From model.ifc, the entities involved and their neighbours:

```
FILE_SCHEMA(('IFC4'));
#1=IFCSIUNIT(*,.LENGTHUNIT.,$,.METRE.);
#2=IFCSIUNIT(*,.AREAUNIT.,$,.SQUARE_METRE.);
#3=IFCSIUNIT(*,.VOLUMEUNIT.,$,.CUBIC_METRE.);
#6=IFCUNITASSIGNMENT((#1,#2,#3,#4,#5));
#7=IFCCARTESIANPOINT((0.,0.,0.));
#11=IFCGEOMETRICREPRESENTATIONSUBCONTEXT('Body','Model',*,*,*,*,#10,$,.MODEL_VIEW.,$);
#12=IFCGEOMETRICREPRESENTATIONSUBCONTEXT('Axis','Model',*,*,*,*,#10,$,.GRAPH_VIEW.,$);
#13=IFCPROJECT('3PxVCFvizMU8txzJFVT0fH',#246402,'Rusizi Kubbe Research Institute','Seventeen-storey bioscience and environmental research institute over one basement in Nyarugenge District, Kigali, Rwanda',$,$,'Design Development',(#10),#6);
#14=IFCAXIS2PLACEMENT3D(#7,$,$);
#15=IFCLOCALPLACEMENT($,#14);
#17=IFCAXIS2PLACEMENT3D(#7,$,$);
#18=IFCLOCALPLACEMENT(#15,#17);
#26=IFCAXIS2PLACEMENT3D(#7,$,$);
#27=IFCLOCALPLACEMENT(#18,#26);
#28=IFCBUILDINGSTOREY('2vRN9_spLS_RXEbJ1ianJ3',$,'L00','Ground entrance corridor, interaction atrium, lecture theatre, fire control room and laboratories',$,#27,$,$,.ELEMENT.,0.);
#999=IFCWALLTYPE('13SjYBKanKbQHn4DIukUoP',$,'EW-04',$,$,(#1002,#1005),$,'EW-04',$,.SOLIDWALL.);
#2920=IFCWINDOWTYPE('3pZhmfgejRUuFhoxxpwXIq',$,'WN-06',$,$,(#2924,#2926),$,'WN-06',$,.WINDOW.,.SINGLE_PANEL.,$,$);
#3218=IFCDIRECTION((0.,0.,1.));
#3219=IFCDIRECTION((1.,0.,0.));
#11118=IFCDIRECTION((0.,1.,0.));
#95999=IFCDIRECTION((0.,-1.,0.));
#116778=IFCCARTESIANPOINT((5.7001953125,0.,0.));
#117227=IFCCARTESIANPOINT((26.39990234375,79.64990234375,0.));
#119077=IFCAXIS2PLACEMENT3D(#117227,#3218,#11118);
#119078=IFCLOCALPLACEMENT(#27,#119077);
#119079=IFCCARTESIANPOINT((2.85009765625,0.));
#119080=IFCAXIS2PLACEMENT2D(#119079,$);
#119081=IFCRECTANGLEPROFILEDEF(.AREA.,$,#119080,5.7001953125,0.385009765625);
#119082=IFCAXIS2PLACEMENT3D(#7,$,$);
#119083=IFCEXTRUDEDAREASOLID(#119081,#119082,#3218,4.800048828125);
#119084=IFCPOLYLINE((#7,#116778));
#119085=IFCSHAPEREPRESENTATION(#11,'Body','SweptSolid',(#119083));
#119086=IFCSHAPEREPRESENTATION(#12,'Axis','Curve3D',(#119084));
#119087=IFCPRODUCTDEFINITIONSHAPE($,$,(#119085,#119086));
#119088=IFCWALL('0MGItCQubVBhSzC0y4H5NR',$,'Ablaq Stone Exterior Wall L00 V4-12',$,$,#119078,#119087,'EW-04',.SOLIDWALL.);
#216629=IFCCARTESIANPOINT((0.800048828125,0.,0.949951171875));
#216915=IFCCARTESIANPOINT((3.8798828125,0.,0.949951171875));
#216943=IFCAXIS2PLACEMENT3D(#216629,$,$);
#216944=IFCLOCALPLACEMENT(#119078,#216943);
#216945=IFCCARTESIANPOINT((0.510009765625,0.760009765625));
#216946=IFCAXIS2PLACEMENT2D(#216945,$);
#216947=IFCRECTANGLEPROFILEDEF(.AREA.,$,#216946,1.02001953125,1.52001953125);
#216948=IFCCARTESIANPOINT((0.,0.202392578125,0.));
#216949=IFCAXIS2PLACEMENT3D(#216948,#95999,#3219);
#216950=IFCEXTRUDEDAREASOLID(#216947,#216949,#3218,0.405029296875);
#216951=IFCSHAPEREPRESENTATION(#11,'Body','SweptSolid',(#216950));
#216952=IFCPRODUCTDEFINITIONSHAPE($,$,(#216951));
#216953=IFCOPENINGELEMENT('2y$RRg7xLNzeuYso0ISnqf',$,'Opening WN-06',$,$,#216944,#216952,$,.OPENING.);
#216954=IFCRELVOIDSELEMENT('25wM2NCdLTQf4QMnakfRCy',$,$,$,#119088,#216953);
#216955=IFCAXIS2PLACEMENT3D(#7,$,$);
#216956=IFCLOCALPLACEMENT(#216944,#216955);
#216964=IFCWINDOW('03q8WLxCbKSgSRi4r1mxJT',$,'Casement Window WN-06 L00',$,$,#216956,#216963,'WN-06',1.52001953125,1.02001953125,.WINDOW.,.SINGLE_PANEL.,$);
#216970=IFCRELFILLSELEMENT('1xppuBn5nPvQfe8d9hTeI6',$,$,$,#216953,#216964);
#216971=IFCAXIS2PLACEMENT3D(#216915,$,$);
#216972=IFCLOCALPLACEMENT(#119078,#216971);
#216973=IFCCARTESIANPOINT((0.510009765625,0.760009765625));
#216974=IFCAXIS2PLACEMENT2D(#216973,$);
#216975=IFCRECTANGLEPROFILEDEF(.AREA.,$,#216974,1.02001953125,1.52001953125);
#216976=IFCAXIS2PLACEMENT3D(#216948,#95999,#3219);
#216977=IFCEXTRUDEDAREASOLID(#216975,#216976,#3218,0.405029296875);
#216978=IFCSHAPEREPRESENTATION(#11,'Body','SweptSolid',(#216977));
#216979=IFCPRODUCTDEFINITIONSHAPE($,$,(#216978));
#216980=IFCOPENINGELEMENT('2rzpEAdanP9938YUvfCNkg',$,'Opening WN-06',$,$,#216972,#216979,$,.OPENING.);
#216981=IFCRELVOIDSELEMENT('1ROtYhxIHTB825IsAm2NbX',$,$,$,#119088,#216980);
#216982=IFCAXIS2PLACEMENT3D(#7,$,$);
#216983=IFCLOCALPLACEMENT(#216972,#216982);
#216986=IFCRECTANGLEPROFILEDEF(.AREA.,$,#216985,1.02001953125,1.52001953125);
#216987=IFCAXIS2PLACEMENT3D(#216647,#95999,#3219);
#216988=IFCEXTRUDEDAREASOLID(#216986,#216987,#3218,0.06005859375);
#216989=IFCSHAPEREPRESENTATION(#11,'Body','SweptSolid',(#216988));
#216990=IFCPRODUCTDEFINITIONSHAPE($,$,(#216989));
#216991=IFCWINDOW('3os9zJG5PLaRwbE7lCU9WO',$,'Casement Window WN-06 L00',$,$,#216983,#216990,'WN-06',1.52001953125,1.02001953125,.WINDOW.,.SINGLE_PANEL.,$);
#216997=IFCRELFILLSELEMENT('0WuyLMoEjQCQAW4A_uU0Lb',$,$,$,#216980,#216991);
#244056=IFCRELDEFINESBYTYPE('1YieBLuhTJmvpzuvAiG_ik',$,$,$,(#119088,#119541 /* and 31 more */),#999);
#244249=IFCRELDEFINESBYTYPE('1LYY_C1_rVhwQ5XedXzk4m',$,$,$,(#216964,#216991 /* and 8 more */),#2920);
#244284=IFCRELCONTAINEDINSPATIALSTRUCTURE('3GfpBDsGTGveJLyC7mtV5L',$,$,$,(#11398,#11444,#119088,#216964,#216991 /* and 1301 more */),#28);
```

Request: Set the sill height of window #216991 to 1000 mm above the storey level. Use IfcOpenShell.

```python
import numpy as np
import ifcopenshell
import ifcopenshell.api.geometry
import ifcopenshell.geom
import ifcopenshell.util.element
import ifcopenshell.util.placement
import ifcopenshell.util.shape
import ifcopenshell.util.unit

model = ifcopenshell.open("model.ifc")
unit_scale = ifcopenshell.util.unit.calculate_unit_scale(model)

window = model.by_guid("3os9zJG5PLaRwbE7lCU9WO")
opening = window.FillsVoids[0].RelatingOpeningElement
storey = ifcopenshell.util.element.get_container(window, ifc_class="IfcBuildingStorey")
level = ifcopenshell.util.placement.get_local_placement(storey.ObjectPlacement)[2, 3]

# The opening's origin need not be at the sill, so measure its lowest point.
shape = ifcopenshell.geom.create_shape(ifcopenshell.geom.settings(), opening)
bottom = ifcopenshell.util.shape.get_shape_bottom_elevation(shape, shape.geometry) / unit_scale
dz = level + 1 / unit_scale - bottom

shift = np.array([0.0, 0.0, dz])
# The window is placed relative to its opening, so it follows when the opening moves.
matrix = ifcopenshell.util.placement.get_local_placement(opening.ObjectPlacement)
matrix[:3, 3] += shift
ifcopenshell.api.geometry.edit_object_placement(
    model, product=opening, matrix=matrix, is_si=False, should_transform_children=True
)

print(f"moved by {dz * unit_scale:+.3f} m")

model.write("model_updated.ifc")
```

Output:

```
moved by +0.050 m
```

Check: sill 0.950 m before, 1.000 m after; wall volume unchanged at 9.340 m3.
